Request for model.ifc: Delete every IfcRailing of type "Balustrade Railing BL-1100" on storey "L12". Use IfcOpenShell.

First a look at what the model holds.

```python
import ifcopenshell
import ifcopenshell.util.element

model = ifcopenshell.open("model.ifc")
print(model.schema)
storey = next(s for s in model.by_type("IfcBuildingStorey") if s.Name == "L12")
railings = [e for e in ifcopenshell.util.element.get_decomposition(storey) if e.is_a("IfcRailing")]
seen = {}
for e in railings:
    element_type = ifcopenshell.util.element.get_type(e)
    name = element_type.Name if element_type not in (None, e) else None
    seen[name] = seen.get(name, 0) + 1
for name, count in sorted(seen.items(), key=str):
    print(count, "x", name)
```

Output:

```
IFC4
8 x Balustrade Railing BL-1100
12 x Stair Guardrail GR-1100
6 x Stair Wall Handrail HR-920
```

```python
import ifcopenshell
import ifcopenshell.api.root
import ifcopenshell.util.element

model = ifcopenshell.open("model.ifc")

storey = next(s for s in model.by_type("IfcBuildingStorey") if s.Name == "L12")
railings = [e for e in ifcopenshell.util.element.get_decomposition(storey) if e.is_a("IfcRailing")]
targets = [e for e in railings if (t := ifcopenshell.util.element.get_type(e)) not in (None, e) and t.Name == "Balustrade Railing BL-1100"]

for e in targets:
    ifcopenshell.api.root.remove_product(model, product=e)
print(len(targets), "removed")

model.write("model_rev.ifc")
```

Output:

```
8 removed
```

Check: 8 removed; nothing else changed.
